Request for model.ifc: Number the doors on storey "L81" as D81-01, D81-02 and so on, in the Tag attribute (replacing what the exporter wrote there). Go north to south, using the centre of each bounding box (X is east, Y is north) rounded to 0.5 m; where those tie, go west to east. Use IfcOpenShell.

First a look at what the model holds.

```python
import ifcopenshell
import ifcopenshell.util.element
import ifcopenshell.util.placement

model = ifcopenshell.open("model.ifc")
print(model.schema)
storey = next(s for s in model.by_type("IfcBuildingStorey") if s.Name == "L81")
doors = [e for e in ifcopenshell.util.element.get_decomposition(storey) if e.is_a("IfcDoor")]
for e in sorted(doors, key=lambda e: e.id()):
    origin = ifcopenshell.util.placement.get_local_placement(e.ObjectPlacement)[:3, 3]
    print(e.id(), e.Tag, e.Name, origin.round(2) + 0.0, sep=" | ")
```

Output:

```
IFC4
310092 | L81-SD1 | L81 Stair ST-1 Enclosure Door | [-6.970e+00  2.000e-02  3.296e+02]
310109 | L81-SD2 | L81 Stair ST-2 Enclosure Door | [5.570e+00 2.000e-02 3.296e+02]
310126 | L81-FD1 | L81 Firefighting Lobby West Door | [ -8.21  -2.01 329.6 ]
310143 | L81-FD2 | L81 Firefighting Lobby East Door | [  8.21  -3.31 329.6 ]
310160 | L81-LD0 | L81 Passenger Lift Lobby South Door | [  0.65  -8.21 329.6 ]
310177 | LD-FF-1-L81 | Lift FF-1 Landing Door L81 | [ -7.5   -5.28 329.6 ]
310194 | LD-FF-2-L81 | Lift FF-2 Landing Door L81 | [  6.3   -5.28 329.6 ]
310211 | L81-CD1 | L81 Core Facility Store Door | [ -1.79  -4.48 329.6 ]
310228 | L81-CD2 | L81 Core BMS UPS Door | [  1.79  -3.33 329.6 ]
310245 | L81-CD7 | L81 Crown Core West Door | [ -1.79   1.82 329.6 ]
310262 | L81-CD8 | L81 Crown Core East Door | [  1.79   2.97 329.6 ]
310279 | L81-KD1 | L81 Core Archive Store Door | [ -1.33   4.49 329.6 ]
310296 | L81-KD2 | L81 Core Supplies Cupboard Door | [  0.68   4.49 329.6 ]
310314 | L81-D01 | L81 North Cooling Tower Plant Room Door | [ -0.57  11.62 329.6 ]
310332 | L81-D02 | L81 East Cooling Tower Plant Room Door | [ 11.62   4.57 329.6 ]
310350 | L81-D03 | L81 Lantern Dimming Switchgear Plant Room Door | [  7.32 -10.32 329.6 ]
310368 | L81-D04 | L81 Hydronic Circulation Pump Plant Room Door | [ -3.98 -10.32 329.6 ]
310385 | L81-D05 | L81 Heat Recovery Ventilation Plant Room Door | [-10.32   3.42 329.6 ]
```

```python
import ifcopenshell
import ifcopenshell.geom
import ifcopenshell.util.element
import ifcopenshell.util.shape

model = ifcopenshell.open("model.ifc")
settings = ifcopenshell.geom.settings()
settings.set("use-world-coords", True)


def centre(element):
    shape = ifcopenshell.geom.create_shape(settings, element)
    return ifcopenshell.util.shape.get_bbox_centroid(shape.geometry)


storey = next(s for s in model.by_type("IfcBuildingStorey") if s.Name == "L81")
doors = [e for e in ifcopenshell.util.element.get_decomposition(storey) if e.is_a("IfcDoor")]

# Insertion points can sit at a corner or the storey origin, so sort by the geometry (in metres).
centres = {e: centre(e) for e in doors}
doors.sort(key=lambda e: (-round(centres[e][1] / 0.5), centres[e][0]))

for i, e in enumerate(doors, start=1):
    number = f"D81-{i:02d}"
    e.Tag = number
    print(e.id(), number)

model.write("model_rev.ifc")
```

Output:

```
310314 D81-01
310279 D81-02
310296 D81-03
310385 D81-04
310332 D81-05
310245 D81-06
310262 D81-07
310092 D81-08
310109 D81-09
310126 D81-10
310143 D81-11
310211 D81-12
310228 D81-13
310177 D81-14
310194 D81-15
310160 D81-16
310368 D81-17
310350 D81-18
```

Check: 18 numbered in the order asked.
